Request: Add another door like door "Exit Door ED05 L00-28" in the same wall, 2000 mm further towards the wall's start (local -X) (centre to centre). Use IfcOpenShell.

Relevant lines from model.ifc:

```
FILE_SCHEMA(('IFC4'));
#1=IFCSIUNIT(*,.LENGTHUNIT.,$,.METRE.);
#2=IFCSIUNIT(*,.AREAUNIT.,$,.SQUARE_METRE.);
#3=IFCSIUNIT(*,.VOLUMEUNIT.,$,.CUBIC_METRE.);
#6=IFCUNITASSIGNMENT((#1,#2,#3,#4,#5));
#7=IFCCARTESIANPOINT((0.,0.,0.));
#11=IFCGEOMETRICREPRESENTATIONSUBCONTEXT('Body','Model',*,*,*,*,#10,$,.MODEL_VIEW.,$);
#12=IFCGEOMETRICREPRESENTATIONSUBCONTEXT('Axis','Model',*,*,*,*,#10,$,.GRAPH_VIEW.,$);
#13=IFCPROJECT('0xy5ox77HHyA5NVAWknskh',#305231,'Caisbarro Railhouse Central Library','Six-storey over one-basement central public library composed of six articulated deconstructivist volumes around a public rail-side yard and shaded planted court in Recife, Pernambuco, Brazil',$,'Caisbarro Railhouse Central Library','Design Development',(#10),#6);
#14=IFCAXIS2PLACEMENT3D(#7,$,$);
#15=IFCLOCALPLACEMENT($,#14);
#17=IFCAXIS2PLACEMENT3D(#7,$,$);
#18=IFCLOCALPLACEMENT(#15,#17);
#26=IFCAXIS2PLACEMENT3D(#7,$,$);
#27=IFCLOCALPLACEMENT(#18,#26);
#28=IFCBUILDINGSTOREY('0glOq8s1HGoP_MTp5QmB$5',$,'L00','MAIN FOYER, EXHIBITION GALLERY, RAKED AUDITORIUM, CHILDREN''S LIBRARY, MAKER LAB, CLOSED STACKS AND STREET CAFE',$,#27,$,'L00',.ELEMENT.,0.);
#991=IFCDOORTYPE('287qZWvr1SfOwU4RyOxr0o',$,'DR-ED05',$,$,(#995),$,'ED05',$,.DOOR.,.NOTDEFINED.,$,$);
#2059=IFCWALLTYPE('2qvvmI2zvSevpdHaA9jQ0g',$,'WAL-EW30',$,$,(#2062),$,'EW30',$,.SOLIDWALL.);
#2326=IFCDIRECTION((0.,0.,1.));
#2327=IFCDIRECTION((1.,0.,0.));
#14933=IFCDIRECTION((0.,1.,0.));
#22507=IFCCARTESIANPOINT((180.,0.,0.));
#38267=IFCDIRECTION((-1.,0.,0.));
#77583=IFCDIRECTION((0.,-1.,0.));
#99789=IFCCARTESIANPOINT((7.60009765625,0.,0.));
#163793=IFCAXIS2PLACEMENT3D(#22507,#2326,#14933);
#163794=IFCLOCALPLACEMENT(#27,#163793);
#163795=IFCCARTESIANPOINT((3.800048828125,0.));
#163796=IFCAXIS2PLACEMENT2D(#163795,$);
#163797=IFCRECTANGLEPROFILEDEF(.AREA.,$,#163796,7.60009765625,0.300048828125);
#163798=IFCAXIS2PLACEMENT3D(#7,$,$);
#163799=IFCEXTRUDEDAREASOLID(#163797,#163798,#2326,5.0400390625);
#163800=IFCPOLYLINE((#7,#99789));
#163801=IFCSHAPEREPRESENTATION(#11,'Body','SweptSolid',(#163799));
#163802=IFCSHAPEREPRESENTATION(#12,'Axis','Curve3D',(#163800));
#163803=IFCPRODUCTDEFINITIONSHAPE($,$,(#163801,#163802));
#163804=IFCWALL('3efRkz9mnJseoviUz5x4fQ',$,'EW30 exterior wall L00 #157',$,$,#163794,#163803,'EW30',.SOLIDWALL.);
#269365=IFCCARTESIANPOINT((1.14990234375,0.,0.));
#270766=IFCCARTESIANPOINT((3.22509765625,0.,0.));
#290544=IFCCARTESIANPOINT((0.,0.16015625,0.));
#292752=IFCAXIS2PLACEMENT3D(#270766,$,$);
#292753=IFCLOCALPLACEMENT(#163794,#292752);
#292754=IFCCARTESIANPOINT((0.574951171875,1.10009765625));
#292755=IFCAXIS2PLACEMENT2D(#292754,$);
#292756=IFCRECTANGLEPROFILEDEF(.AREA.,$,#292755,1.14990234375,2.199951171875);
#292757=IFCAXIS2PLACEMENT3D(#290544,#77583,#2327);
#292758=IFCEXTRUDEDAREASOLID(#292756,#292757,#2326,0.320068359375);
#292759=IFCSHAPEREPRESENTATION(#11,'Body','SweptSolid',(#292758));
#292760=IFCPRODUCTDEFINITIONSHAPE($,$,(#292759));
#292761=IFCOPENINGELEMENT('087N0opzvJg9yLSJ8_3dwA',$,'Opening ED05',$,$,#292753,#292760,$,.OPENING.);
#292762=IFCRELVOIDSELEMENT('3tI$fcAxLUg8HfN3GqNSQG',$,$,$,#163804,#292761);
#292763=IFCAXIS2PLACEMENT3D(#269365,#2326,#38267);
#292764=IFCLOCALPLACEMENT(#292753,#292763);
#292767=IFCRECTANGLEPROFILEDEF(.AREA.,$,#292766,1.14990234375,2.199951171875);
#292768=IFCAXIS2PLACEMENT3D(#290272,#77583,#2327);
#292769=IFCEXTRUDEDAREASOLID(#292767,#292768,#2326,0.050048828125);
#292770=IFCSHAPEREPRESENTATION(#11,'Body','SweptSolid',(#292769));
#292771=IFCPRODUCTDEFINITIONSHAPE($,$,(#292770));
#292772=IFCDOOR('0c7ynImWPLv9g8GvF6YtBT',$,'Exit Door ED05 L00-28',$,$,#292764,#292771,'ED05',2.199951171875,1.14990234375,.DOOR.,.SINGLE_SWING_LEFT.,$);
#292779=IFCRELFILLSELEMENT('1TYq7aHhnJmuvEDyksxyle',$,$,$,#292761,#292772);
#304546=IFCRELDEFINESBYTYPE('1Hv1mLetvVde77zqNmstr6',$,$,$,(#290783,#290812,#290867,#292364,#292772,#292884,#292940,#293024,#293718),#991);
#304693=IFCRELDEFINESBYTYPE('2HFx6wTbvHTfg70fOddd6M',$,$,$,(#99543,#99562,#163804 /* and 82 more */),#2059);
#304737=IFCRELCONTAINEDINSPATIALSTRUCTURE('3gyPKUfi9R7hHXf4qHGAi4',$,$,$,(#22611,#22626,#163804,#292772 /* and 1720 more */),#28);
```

```python
import ifcopenshell
import ifcopenshell.api.feature
import ifcopenshell.api.geometry
import ifcopenshell.api.root
import ifcopenshell.geom
import ifcopenshell.util.element
import ifcopenshell.util.placement
import ifcopenshell.util.shape
import ifcopenshell.util.unit

model = ifcopenshell.open("model.ifc")
unit_scale = ifcopenshell.util.unit.calculate_unit_scale(model)
settings = ifcopenshell.geom.settings()


def volume(element):
    """Net volume in cubic metres, openings subtracted."""
    shape = ifcopenshell.geom.create_shape(settings, element)
    return ifcopenshell.util.shape.get_volume(shape.geometry)


door = model.by_guid("0c7ynImWPLv9g8GvF6YtBT")
opening = door.FillsVoids[0].RelatingOpeningElement
wall = opening.VoidsElements[0].RelatingBuildingElement
before = volume(wall)
shift = ifcopenshell.util.placement.get_local_placement(wall.ObjectPlacement)[:3, 0] * -2 / unit_scale

# copy_class copies the void relationship, type, container and properties, but no geometry.
new_opening = ifcopenshell.api.root.copy_class(model, product=opening)
new_opening.Representation = ifcopenshell.util.element.copy_deep(
    model, opening.Representation, exclude=["IfcGeometricRepresentationContext", "IfcRepresentationMap"]
)
new_door = ifcopenshell.api.root.copy_class(model, product=door)
new_door.Representation = ifcopenshell.util.element.copy_deep(
    model, door.Representation, exclude=["IfcGeometricRepresentationContext", "IfcRepresentationMap"]
)
new_door.Tag = None
ifcopenshell.api.feature.add_filling(model, opening=new_opening, element=new_door)

for old, new in ((opening, new_opening), (door, new_door)):
    matrix = ifcopenshell.util.placement.get_local_placement(old.ObjectPlacement)
    matrix[:3, 3] += shift
    ifcopenshell.api.geometry.edit_object_placement(model, product=new, matrix=matrix, is_si=False)

after = volume(wall)

print(f"wall volume {before:.3f} -> {after:.3f} m3")

model.write("model_rev.ifc")
```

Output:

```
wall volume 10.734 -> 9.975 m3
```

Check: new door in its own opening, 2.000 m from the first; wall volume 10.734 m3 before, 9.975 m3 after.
